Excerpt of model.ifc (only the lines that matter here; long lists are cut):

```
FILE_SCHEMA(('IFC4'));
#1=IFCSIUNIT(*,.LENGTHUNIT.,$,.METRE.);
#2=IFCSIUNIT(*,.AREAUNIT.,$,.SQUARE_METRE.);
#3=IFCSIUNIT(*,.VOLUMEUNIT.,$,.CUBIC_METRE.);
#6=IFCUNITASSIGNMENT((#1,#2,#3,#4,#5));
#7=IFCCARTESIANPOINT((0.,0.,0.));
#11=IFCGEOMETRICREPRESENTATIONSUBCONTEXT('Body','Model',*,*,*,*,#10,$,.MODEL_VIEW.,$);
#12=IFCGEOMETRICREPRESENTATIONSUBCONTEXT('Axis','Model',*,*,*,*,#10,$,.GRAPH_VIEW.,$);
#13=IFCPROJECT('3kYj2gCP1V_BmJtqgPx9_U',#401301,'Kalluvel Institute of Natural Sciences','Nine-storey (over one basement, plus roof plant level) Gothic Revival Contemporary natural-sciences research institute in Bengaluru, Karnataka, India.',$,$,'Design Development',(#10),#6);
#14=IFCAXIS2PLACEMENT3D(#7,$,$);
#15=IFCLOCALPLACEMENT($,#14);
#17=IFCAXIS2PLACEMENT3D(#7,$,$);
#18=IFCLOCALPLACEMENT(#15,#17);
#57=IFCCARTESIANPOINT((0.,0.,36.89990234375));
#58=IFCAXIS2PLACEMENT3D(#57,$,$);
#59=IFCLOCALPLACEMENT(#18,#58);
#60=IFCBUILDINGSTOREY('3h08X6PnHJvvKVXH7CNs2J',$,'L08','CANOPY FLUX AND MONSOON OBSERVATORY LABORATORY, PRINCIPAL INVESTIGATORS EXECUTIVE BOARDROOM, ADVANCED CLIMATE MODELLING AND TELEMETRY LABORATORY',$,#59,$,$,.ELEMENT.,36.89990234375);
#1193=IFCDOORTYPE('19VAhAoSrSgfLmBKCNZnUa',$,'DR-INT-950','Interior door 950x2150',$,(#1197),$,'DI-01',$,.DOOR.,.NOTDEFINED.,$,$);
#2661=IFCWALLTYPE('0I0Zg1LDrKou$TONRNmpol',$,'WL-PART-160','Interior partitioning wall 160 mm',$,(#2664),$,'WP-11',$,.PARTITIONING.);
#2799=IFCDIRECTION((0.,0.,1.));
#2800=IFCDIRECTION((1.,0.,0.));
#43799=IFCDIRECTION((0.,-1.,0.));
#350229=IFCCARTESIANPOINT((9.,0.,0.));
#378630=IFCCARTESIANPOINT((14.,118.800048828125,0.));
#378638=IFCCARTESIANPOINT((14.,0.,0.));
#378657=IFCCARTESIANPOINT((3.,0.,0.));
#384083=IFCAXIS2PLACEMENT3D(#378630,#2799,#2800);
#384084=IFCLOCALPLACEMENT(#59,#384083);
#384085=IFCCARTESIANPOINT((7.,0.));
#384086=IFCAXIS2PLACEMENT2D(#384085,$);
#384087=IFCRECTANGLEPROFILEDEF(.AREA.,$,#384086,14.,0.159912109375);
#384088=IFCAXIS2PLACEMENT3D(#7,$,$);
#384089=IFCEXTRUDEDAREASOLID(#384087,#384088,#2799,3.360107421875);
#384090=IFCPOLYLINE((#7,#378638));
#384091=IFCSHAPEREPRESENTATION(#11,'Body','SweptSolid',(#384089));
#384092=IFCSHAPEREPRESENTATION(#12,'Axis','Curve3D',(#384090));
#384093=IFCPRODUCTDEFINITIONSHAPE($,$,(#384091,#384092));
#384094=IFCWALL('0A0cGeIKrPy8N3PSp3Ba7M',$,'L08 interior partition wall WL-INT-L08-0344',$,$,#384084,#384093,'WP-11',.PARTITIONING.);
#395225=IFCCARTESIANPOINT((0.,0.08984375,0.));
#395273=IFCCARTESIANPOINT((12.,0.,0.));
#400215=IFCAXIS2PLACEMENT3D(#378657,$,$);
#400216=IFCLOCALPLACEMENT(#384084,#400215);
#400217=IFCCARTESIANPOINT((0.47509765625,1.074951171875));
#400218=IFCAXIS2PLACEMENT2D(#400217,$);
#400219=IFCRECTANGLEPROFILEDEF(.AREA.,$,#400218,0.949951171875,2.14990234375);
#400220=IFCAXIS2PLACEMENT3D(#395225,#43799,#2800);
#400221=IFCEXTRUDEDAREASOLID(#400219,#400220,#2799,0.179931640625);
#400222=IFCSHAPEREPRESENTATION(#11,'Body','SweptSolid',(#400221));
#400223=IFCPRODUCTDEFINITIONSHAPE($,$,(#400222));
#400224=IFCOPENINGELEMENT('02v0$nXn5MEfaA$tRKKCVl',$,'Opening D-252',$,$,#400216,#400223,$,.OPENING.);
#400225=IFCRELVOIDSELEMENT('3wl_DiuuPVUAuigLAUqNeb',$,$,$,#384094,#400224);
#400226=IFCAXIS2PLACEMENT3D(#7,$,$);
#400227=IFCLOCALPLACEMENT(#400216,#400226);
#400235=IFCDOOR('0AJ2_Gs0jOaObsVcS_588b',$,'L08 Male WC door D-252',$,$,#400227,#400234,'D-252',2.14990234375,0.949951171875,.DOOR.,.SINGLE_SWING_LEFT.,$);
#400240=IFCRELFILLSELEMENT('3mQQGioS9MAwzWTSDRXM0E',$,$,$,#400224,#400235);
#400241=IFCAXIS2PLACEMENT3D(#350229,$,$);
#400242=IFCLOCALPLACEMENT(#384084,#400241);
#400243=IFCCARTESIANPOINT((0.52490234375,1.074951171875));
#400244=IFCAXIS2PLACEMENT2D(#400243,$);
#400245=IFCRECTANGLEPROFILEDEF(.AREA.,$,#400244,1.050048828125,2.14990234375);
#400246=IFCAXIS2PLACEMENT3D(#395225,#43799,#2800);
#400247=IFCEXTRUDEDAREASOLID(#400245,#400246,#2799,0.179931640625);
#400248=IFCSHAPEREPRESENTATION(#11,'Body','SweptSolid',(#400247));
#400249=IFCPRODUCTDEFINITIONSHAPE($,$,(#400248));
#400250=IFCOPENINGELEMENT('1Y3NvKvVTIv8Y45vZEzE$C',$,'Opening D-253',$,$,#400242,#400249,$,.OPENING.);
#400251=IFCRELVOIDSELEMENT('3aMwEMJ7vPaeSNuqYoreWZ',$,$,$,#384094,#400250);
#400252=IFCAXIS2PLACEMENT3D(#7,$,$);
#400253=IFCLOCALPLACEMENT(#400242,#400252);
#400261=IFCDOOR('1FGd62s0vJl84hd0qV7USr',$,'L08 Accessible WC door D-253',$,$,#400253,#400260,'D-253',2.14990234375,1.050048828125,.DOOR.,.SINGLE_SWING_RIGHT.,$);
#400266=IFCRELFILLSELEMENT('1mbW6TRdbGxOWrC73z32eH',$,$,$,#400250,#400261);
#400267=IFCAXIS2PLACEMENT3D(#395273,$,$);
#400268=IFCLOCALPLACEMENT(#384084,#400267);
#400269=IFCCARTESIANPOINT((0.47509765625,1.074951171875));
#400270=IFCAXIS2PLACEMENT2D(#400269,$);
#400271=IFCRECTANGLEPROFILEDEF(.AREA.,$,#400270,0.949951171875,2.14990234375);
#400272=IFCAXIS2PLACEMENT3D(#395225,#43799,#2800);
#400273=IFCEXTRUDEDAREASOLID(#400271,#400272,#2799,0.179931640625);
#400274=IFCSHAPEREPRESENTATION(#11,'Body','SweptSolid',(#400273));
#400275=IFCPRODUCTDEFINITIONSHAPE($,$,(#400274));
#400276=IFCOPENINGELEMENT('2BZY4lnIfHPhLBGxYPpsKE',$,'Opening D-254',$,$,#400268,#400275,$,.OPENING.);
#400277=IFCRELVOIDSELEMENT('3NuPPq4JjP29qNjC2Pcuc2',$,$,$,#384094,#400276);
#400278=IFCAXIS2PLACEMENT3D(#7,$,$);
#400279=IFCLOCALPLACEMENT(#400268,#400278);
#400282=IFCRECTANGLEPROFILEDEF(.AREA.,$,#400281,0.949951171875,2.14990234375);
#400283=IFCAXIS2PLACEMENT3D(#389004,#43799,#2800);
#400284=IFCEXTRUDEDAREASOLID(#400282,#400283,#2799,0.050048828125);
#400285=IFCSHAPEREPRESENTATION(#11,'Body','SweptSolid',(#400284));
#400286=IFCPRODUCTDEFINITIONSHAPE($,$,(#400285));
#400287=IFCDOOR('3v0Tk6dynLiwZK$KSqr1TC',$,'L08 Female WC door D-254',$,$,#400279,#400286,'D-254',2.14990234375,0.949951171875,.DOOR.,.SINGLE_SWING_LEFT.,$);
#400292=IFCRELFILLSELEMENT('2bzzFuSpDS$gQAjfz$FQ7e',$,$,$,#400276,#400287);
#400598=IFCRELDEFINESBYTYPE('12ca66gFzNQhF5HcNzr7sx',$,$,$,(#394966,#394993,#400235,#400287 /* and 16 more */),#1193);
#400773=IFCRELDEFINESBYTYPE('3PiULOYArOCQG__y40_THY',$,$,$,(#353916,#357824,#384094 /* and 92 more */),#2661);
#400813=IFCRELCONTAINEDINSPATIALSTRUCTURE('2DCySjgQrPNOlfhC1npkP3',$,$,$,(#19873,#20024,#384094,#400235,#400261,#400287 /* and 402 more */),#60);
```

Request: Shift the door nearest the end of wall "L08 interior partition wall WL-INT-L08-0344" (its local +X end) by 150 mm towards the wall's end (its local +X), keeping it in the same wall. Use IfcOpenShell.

```python
import ifcopenshell
import ifcopenshell.api.geometry
import ifcopenshell.util.placement

model = ifcopenshell.open("model.ifc")

door = model.by_guid("3v0Tk6dynLiwZK$KSqr1TC")
opening = door.FillsVoids[0].RelatingOpeningElement
wall = opening.VoidsElements[0].RelatingBuildingElement

wall_matrix = ifcopenshell.util.placement.get_local_placement(wall.ObjectPlacement)
shift = wall_matrix[:3, 0] * 0.15
before = ifcopenshell.util.placement.get_local_placement(door.ObjectPlacement)[:3, 3].copy()

# The door is placed relative to its opening, so it follows when the opening moves.
matrix = ifcopenshell.util.placement.get_local_placement(opening.ObjectPlacement)
matrix[:3, 3] += shift
ifcopenshell.api.geometry.edit_object_placement(
    model, product=opening, matrix=matrix, is_si=False, should_transform_children=True
)

after = ifcopenshell.util.placement.get_local_placement(door.ObjectPlacement)[:3, 3]
print("door moved by", (after - before).round(3) + 0.0)

model.write("model_v2.ifc")
```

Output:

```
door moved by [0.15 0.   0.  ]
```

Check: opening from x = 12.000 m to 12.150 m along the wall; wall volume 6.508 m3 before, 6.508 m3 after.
